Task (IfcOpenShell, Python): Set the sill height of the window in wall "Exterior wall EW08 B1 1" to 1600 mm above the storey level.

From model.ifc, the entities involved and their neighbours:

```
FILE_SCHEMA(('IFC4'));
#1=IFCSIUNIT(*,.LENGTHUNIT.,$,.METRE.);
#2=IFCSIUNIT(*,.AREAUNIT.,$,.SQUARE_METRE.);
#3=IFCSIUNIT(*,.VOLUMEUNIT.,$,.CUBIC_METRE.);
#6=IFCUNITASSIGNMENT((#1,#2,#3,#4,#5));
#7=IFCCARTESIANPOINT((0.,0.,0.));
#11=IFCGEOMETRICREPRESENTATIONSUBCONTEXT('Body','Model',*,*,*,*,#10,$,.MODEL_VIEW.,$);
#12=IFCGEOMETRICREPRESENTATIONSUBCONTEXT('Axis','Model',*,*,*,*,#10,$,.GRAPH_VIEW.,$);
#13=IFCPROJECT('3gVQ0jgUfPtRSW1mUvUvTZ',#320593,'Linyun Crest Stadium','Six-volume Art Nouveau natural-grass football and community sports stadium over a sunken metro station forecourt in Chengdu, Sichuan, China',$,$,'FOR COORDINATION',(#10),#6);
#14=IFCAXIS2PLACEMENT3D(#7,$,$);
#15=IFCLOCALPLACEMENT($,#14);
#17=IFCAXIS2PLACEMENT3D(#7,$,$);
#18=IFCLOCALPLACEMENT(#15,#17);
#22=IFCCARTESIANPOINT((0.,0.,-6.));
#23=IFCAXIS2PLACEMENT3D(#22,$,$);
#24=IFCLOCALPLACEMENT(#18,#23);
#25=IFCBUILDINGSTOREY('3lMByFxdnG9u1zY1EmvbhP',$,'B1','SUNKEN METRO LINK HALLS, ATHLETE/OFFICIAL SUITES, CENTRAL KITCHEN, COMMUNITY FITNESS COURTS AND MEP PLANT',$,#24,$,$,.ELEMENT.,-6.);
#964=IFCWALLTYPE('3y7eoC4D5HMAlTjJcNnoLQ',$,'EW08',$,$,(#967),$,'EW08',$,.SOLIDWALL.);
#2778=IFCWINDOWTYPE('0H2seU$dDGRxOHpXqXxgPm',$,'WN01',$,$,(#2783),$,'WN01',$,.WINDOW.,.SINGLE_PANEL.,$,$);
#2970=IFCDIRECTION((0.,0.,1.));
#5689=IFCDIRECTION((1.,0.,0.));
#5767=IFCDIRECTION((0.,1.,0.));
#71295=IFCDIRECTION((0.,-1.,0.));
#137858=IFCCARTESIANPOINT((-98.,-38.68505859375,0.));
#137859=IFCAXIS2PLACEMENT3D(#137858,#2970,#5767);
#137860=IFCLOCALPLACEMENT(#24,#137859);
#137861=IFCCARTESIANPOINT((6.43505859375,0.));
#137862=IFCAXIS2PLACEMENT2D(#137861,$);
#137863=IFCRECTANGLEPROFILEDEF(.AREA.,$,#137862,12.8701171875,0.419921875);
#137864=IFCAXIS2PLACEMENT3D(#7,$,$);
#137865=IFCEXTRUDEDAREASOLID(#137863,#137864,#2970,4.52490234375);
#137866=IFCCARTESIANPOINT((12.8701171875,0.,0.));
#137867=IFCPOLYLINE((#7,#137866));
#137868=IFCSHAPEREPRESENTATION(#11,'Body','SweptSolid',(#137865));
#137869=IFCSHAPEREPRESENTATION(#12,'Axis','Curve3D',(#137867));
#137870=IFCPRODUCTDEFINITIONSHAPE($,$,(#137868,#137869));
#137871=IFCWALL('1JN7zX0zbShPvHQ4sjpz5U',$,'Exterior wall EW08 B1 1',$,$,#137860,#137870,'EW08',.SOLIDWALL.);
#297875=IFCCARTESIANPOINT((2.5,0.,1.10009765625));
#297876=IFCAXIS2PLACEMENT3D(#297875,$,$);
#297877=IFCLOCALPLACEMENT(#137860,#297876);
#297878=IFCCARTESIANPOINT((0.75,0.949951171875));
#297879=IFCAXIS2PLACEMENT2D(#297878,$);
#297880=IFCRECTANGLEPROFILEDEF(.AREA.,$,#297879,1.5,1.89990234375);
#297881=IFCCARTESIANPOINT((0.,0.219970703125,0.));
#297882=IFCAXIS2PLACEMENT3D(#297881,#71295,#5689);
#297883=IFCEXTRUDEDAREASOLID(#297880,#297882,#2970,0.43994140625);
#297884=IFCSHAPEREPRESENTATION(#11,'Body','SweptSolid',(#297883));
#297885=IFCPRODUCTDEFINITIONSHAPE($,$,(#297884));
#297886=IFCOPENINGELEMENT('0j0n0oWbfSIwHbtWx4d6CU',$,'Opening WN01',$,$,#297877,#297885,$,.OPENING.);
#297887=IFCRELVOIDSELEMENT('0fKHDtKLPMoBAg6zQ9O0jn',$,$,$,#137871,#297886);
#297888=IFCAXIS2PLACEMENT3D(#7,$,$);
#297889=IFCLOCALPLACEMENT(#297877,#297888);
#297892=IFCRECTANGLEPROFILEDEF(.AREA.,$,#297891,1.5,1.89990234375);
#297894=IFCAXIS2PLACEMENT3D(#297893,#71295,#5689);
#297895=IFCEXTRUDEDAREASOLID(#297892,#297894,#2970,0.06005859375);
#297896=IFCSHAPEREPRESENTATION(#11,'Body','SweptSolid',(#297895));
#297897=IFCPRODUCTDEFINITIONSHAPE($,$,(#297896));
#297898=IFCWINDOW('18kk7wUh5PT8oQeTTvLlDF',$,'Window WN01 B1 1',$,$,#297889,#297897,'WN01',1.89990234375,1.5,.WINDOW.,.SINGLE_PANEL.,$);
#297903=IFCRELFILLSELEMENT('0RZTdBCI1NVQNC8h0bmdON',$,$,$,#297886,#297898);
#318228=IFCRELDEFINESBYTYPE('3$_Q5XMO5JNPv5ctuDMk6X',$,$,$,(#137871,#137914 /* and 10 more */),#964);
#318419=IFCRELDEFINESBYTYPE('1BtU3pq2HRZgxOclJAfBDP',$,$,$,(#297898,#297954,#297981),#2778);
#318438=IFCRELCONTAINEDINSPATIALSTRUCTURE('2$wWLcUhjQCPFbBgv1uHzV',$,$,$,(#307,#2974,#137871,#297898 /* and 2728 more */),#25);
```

```python
import numpy as np
import ifcopenshell
import ifcopenshell.api.geometry
import ifcopenshell.geom
import ifcopenshell.util.element
import ifcopenshell.util.placement
import ifcopenshell.util.shape
import ifcopenshell.util.unit

model = ifcopenshell.open("model.ifc")
unit_scale = ifcopenshell.util.unit.calculate_unit_scale(model)

window = model.by_id(297898)
opening = window.FillsVoids[0].RelatingOpeningElement
storey = ifcopenshell.util.element.get_container(window, ifc_class="IfcBuildingStorey")
level = ifcopenshell.util.placement.get_local_placement(storey.ObjectPlacement)[2, 3]

# The opening's origin need not be at the sill, so measure its lowest point.
shape = ifcopenshell.geom.create_shape(ifcopenshell.geom.settings(), opening)
bottom = ifcopenshell.util.shape.get_shape_bottom_elevation(shape, shape.geometry) / unit_scale
dz = level + 1.6 / unit_scale - bottom

shift = np.array([0.0, 0.0, dz])
# The window is placed relative to its opening, so it follows when the opening moves.
matrix = ifcopenshell.util.placement.get_local_placement(opening.ObjectPlacement)
matrix[:3, 3] += shift
ifcopenshell.api.geometry.edit_object_placement(
    model, product=opening, matrix=matrix, is_si=False, should_transform_children=True
)

print(f"moved by {dz * unit_scale:+.3f} m")

model.write("model_rev.ifc")
```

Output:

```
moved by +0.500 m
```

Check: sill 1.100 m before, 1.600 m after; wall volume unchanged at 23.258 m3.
